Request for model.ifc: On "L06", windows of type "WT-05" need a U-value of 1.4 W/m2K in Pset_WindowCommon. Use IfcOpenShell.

First a look at what the model holds.

```python
import ifcopenshell
import ifcopenshell.util.element

model = ifcopenshell.open("model.ifc")
print(model.schema)
storey = next(s for s in model.by_type("IfcBuildingStorey") if s.Name == "L06")
windows = [e for e in ifcopenshell.util.element.get_decomposition(storey) if e.is_a("IfcWindow")]
seen = {}
for e in windows:
    element_type = ifcopenshell.util.element.get_type(e)
    key = (element_type.Name if element_type != e and element_type else None, ifcopenshell.util.element.get_pset(e, "Pset_WindowCommon", "ThermalTransmittance"))
    seen[key] = seen.get(key, 0) + 1
for (name, value), count in sorted(seen.items(), key=str):
    print(count, "x", name, "|", value)
```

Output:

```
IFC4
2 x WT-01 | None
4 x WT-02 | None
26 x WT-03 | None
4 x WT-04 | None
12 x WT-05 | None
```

```python
import ifcopenshell
import ifcopenshell.api.pset
import ifcopenshell.util.element

model = ifcopenshell.open("model.ifc")

storey = next(s for s in model.by_type("IfcBuildingStorey") if s.Name == "L06")
windows = [e for e in ifcopenshell.util.element.get_decomposition(storey) if e.is_a("IfcWindow")]

count = 0
for e in windows:
    element_type = ifcopenshell.util.element.get_type(e)
    if element_type in (None, e) or element_type.Name != "WT-05":
        continue
    # add_pset returns the element's existing set when there is one.
    pset = ifcopenshell.api.pset.add_pset(model, product=e, name="Pset_WindowCommon")
    ifcopenshell.api.pset.edit_pset(model, pset=pset, properties={"ThermalTransmittance": 1.4})
    count += 1

print(count, "windows updated")

model.write("model_v2.ifc")
```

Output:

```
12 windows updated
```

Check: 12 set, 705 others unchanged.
